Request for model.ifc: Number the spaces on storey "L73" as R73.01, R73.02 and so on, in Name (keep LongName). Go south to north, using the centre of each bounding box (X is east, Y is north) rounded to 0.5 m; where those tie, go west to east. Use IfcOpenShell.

First a look at what the model holds.

```python
import ifcopenshell
import ifcopenshell.util.element
import ifcopenshell.util.placement

model = ifcopenshell.open("model.ifc")
print(model.schema)
storey = next(s for s in model.by_type("IfcBuildingStorey") if s.Name == "L73")
spaces = [e for e in ifcopenshell.util.element.get_decomposition(storey) if e.is_a("IfcSpace")]
for e in sorted(spaces, key=lambda e: e.id()):
    origin = ifcopenshell.util.placement.get_local_placement(e.ObjectPlacement)[:3, 3]
    print(e.id(), e.Name, e.LongName, origin.round(2) + 0.0, sep=" | ")
```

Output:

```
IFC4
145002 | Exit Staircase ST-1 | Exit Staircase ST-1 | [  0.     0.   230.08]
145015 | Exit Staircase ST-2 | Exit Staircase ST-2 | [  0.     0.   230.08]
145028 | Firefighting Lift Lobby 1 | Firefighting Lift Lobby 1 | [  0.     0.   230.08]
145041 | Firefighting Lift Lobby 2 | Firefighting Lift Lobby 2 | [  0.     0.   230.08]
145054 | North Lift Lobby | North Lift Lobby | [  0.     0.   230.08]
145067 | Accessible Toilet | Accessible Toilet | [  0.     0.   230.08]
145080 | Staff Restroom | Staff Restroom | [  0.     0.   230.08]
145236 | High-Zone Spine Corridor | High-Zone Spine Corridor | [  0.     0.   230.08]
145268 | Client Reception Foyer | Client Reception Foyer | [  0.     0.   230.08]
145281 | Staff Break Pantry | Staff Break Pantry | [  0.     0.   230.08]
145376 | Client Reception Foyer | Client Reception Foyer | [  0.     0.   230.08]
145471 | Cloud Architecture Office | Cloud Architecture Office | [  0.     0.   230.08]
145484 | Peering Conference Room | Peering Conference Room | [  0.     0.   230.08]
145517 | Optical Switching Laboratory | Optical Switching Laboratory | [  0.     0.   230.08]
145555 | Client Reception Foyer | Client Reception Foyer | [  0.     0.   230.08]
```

```python
import ifcopenshell
import ifcopenshell.geom
import ifcopenshell.util.element
import ifcopenshell.util.shape

model = ifcopenshell.open("model.ifc")
settings = ifcopenshell.geom.settings()
settings.set("use-world-coords", True)


def centre(element):
    shape = ifcopenshell.geom.create_shape(settings, element)
    return ifcopenshell.util.shape.get_bbox_centroid(shape.geometry)


storey = next(s for s in model.by_type("IfcBuildingStorey") if s.Name == "L73")
spaces = [e for e in ifcopenshell.util.element.get_decomposition(storey) if e.is_a("IfcSpace")]

# Insertion points can sit at a corner or the storey origin, so sort by the geometry (in metres).
centres = {e: centre(e) for e in spaces}
spaces.sort(key=lambda e: (round(centres[e][1] / 0.5), centres[e][0]))

for i, e in enumerate(spaces, start=1):
    number = f"R73.{i:02d}"
    e.Name = number
    print(e.id(), number)

model.write("model_v2.ifc")
```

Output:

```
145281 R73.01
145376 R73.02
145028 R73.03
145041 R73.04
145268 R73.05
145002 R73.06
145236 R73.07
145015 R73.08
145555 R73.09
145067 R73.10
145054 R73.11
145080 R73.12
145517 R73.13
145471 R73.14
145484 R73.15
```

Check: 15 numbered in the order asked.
